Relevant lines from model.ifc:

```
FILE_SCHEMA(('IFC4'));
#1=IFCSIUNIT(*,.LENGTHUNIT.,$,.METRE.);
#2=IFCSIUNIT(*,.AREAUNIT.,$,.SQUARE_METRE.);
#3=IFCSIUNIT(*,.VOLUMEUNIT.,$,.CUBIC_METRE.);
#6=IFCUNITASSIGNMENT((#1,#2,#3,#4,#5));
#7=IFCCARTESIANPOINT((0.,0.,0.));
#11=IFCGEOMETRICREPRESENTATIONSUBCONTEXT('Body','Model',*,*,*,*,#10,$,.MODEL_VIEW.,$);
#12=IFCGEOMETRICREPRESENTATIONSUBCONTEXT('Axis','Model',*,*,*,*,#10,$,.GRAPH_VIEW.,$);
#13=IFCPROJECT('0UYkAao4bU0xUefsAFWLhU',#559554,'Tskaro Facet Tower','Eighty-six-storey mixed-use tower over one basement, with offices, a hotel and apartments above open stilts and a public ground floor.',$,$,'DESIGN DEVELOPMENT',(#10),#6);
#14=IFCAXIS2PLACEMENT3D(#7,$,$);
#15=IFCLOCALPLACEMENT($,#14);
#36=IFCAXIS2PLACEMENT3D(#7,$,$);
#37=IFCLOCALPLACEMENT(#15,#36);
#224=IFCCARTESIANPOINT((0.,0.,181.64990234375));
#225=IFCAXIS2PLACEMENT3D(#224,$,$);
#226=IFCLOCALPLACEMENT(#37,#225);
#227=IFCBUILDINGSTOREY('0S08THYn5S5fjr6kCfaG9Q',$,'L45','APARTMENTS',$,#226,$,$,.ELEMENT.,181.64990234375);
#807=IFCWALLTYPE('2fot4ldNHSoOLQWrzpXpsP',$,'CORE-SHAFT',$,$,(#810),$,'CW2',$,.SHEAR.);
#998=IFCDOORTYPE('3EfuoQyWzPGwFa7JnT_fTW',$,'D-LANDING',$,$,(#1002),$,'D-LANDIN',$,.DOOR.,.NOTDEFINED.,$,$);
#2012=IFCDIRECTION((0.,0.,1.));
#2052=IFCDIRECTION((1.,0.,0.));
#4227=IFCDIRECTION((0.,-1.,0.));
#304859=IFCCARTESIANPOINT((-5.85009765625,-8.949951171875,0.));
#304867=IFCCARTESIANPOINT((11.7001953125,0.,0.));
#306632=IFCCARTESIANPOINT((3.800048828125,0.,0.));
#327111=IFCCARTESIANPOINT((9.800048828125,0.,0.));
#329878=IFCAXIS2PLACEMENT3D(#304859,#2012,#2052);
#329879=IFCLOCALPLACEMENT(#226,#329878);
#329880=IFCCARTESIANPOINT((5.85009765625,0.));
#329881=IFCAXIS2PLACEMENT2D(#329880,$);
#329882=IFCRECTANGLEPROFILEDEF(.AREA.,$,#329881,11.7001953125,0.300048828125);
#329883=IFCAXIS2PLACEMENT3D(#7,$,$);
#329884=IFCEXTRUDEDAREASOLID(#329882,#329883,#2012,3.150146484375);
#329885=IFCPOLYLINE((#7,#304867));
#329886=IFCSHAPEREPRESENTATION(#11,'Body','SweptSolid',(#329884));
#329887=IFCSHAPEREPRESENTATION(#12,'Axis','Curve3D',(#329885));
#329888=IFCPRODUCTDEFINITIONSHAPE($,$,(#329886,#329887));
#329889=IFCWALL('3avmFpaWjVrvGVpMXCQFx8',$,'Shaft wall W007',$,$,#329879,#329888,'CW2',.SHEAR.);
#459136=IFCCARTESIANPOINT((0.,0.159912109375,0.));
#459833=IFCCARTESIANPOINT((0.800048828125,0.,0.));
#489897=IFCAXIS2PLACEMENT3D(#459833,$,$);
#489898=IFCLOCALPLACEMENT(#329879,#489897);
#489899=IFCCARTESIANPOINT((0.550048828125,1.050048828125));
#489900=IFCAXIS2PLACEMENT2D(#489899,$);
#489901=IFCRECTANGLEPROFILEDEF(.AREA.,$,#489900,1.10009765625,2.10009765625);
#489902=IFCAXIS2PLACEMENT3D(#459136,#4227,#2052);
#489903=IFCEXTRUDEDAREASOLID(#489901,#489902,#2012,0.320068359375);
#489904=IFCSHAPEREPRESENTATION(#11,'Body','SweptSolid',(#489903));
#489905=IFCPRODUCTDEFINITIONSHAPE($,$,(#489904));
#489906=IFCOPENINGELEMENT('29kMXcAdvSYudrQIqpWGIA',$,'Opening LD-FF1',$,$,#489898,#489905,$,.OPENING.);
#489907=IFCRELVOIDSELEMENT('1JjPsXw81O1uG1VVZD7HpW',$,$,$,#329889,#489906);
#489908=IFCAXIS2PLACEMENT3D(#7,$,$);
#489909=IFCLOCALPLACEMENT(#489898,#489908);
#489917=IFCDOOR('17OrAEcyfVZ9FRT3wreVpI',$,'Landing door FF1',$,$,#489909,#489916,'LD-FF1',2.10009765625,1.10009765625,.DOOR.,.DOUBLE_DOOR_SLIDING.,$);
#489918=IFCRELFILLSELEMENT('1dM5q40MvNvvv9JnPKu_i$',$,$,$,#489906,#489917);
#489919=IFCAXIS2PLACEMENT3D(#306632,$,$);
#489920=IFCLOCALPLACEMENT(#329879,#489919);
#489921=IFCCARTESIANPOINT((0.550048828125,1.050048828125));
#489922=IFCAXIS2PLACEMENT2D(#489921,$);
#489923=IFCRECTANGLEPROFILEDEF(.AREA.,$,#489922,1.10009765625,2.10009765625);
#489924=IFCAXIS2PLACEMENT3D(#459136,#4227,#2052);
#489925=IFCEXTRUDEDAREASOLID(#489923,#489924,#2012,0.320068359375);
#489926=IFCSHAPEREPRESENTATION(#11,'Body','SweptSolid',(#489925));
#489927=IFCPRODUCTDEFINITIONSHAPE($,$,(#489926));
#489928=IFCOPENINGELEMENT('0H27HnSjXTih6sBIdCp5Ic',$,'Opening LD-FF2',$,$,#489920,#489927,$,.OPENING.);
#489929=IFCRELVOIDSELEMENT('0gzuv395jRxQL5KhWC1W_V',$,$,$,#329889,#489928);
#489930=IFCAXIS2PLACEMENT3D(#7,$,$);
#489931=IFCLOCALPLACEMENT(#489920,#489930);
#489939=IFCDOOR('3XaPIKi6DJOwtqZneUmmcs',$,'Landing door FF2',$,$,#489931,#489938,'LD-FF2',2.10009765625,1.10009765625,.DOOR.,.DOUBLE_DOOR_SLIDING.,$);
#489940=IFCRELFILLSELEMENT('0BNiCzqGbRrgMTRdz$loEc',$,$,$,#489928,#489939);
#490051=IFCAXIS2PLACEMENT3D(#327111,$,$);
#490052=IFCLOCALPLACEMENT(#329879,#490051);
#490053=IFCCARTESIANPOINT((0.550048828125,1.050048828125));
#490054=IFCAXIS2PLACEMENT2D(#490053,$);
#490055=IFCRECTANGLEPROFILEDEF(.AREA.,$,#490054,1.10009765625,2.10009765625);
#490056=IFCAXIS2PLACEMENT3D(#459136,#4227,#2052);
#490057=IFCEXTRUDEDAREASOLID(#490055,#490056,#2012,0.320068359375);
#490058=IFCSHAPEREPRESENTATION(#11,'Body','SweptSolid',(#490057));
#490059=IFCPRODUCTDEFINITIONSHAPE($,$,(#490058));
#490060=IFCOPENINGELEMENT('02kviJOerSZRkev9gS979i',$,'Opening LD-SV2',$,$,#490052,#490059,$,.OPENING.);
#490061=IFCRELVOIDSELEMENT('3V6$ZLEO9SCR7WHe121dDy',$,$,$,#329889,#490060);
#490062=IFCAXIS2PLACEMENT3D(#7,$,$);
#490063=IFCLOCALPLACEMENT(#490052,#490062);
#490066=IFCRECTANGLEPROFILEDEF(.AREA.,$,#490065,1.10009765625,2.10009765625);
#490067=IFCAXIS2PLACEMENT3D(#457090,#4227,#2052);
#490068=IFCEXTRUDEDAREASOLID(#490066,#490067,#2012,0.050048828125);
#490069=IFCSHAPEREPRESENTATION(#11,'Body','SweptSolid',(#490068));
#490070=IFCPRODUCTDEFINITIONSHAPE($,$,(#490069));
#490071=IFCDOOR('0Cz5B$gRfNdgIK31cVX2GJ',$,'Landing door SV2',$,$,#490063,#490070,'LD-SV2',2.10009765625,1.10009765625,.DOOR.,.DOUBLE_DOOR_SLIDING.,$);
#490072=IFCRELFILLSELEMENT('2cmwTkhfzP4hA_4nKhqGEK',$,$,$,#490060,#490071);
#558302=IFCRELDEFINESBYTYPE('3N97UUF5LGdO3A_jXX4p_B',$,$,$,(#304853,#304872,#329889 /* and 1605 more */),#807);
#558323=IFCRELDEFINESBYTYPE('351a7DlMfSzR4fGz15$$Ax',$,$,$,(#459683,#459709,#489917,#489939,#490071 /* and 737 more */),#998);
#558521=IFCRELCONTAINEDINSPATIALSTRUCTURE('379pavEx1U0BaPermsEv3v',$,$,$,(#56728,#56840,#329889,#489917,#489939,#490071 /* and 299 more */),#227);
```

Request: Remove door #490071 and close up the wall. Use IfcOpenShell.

```python
import ifcopenshell
import ifcopenshell.api.feature
import ifcopenshell.api.root
import ifcopenshell.geom
import ifcopenshell.util.shape

model = ifcopenshell.open("model.ifc")
settings = ifcopenshell.geom.settings()


def volume(element):
    """Net volume in cubic metres, openings subtracted."""
    shape = ifcopenshell.geom.create_shape(settings, element)
    return ifcopenshell.util.shape.get_volume(shape.geometry)


door = model.by_guid("0Cz5B$gRfNdgIK31cVX2GJ")
opening = door.FillsVoids[0].RelatingOpeningElement
wall = opening.VoidsElements[0].RelatingBuildingElement
before = volume(wall)

ifcopenshell.api.root.remove_product(model, product=door)
ifcopenshell.api.feature.remove_feature(model, feature=opening)

after = volume(wall)

print(f"wall volume {before:.3f} -> {after:.3f} m3")

model.write("model-out.ifc")
```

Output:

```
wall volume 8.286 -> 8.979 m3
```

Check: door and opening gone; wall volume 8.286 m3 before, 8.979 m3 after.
